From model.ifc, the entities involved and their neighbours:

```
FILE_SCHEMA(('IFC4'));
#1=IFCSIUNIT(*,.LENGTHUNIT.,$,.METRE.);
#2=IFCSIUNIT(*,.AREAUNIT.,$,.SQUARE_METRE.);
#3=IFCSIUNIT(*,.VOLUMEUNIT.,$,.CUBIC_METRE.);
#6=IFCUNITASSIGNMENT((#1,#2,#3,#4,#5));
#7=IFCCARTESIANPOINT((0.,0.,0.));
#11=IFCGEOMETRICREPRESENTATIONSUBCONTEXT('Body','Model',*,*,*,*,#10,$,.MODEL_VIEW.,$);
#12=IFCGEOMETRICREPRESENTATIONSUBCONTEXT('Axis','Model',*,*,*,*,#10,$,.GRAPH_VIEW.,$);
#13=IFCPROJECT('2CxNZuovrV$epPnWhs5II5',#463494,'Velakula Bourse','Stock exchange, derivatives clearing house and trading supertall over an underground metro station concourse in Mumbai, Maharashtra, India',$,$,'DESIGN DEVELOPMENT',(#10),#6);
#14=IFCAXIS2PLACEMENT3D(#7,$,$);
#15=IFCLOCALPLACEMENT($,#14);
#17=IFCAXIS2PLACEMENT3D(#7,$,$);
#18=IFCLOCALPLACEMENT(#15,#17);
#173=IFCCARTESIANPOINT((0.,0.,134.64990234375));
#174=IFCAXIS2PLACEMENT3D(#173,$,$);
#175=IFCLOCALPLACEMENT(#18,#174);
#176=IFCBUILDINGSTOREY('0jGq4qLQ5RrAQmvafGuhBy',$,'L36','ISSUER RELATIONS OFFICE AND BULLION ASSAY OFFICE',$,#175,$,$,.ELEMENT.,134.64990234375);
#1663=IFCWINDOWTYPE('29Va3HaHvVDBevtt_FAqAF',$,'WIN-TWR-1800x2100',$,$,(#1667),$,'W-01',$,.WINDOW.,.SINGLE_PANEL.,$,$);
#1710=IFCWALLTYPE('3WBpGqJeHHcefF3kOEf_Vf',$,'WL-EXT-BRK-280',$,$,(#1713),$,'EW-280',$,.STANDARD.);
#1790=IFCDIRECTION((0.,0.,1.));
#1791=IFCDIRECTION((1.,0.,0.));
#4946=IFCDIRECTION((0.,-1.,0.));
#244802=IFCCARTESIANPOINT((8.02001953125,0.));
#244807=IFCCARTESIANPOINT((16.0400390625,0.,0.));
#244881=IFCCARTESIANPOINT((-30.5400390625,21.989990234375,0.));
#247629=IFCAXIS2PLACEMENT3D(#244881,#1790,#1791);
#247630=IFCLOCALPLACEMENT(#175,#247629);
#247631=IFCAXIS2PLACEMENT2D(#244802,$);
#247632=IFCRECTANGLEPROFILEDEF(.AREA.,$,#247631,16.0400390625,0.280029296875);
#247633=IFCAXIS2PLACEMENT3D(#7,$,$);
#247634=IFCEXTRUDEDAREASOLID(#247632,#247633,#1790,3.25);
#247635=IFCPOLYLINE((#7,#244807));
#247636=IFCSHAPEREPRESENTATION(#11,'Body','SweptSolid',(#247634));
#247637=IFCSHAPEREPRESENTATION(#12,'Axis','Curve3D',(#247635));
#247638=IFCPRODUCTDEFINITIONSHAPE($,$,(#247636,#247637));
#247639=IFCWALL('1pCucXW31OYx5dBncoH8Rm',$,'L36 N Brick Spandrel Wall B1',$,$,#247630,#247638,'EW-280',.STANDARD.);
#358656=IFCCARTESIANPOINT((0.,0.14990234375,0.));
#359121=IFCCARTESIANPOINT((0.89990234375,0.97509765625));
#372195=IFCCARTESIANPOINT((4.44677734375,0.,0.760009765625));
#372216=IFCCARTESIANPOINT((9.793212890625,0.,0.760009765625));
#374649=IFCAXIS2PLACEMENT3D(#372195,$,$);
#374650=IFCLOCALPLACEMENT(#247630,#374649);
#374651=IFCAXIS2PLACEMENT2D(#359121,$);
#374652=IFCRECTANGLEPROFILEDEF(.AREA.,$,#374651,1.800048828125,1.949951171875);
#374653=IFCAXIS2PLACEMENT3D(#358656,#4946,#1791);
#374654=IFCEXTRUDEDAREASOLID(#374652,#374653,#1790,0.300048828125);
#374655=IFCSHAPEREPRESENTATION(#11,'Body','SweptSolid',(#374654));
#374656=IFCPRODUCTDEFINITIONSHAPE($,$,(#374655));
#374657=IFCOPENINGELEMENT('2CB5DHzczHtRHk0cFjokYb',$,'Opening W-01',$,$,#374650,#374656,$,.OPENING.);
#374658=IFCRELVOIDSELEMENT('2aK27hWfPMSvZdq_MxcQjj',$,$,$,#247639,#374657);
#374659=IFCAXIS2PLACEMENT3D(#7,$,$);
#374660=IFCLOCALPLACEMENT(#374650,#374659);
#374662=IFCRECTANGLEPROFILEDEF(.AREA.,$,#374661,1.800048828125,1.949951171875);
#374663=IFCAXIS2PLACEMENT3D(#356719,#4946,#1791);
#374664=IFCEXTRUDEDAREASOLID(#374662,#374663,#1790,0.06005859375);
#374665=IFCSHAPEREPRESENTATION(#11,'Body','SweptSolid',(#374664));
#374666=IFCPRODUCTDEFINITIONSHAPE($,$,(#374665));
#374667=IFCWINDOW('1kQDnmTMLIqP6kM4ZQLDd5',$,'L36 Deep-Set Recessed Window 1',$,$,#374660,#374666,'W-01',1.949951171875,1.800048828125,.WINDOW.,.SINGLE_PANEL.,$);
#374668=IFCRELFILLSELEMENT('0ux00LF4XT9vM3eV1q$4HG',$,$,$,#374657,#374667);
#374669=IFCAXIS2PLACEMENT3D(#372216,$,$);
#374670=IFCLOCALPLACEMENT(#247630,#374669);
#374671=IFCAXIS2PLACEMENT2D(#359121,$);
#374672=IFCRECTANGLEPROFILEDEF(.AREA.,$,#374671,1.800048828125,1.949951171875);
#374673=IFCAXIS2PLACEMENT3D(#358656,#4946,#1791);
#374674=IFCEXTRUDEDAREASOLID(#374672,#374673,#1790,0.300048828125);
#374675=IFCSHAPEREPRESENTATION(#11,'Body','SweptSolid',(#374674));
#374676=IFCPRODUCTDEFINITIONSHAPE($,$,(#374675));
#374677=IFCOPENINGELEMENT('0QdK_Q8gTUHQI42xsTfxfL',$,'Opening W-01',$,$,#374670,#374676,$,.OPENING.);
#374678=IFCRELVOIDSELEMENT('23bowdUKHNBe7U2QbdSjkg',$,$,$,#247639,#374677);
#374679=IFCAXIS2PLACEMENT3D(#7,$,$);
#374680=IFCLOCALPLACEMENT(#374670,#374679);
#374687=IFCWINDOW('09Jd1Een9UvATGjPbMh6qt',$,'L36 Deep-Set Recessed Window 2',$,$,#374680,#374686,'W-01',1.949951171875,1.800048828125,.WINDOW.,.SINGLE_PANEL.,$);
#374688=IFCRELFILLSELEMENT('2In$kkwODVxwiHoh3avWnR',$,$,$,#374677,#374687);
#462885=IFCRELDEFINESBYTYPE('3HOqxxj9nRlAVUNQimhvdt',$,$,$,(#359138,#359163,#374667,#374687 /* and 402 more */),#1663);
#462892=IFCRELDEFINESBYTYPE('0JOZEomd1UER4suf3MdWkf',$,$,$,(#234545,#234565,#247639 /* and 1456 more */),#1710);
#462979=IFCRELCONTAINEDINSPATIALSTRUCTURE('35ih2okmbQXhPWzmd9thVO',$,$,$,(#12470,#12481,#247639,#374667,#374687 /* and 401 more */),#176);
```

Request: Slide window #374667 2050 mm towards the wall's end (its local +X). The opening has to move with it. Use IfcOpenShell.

```python
import ifcopenshell
import ifcopenshell.api.geometry
import ifcopenshell.util.placement

model = ifcopenshell.open("model.ifc")

window = model.by_id(374667)
opening = window.FillsVoids[0].RelatingOpeningElement
wall = opening.VoidsElements[0].RelatingBuildingElement

wall_matrix = ifcopenshell.util.placement.get_local_placement(wall.ObjectPlacement)
shift = wall_matrix[:3, 0] * 2.05
before = ifcopenshell.util.placement.get_local_placement(window.ObjectPlacement)[:3, 3].copy()

# The window is placed relative to its opening, so it follows when the opening moves.
matrix = ifcopenshell.util.placement.get_local_placement(opening.ObjectPlacement)
matrix[:3, 3] += shift
ifcopenshell.api.geometry.edit_object_placement(
    model, product=opening, matrix=matrix, is_si=False, should_transform_children=True
)

after = ifcopenshell.util.placement.get_local_placement(window.ObjectPlacement)[:3, 3]
print("window moved by", (after - before).round(3) + 0.0)

model.write("model-out.ifc")
```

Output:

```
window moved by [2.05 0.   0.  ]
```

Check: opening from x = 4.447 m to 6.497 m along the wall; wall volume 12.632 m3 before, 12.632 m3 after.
